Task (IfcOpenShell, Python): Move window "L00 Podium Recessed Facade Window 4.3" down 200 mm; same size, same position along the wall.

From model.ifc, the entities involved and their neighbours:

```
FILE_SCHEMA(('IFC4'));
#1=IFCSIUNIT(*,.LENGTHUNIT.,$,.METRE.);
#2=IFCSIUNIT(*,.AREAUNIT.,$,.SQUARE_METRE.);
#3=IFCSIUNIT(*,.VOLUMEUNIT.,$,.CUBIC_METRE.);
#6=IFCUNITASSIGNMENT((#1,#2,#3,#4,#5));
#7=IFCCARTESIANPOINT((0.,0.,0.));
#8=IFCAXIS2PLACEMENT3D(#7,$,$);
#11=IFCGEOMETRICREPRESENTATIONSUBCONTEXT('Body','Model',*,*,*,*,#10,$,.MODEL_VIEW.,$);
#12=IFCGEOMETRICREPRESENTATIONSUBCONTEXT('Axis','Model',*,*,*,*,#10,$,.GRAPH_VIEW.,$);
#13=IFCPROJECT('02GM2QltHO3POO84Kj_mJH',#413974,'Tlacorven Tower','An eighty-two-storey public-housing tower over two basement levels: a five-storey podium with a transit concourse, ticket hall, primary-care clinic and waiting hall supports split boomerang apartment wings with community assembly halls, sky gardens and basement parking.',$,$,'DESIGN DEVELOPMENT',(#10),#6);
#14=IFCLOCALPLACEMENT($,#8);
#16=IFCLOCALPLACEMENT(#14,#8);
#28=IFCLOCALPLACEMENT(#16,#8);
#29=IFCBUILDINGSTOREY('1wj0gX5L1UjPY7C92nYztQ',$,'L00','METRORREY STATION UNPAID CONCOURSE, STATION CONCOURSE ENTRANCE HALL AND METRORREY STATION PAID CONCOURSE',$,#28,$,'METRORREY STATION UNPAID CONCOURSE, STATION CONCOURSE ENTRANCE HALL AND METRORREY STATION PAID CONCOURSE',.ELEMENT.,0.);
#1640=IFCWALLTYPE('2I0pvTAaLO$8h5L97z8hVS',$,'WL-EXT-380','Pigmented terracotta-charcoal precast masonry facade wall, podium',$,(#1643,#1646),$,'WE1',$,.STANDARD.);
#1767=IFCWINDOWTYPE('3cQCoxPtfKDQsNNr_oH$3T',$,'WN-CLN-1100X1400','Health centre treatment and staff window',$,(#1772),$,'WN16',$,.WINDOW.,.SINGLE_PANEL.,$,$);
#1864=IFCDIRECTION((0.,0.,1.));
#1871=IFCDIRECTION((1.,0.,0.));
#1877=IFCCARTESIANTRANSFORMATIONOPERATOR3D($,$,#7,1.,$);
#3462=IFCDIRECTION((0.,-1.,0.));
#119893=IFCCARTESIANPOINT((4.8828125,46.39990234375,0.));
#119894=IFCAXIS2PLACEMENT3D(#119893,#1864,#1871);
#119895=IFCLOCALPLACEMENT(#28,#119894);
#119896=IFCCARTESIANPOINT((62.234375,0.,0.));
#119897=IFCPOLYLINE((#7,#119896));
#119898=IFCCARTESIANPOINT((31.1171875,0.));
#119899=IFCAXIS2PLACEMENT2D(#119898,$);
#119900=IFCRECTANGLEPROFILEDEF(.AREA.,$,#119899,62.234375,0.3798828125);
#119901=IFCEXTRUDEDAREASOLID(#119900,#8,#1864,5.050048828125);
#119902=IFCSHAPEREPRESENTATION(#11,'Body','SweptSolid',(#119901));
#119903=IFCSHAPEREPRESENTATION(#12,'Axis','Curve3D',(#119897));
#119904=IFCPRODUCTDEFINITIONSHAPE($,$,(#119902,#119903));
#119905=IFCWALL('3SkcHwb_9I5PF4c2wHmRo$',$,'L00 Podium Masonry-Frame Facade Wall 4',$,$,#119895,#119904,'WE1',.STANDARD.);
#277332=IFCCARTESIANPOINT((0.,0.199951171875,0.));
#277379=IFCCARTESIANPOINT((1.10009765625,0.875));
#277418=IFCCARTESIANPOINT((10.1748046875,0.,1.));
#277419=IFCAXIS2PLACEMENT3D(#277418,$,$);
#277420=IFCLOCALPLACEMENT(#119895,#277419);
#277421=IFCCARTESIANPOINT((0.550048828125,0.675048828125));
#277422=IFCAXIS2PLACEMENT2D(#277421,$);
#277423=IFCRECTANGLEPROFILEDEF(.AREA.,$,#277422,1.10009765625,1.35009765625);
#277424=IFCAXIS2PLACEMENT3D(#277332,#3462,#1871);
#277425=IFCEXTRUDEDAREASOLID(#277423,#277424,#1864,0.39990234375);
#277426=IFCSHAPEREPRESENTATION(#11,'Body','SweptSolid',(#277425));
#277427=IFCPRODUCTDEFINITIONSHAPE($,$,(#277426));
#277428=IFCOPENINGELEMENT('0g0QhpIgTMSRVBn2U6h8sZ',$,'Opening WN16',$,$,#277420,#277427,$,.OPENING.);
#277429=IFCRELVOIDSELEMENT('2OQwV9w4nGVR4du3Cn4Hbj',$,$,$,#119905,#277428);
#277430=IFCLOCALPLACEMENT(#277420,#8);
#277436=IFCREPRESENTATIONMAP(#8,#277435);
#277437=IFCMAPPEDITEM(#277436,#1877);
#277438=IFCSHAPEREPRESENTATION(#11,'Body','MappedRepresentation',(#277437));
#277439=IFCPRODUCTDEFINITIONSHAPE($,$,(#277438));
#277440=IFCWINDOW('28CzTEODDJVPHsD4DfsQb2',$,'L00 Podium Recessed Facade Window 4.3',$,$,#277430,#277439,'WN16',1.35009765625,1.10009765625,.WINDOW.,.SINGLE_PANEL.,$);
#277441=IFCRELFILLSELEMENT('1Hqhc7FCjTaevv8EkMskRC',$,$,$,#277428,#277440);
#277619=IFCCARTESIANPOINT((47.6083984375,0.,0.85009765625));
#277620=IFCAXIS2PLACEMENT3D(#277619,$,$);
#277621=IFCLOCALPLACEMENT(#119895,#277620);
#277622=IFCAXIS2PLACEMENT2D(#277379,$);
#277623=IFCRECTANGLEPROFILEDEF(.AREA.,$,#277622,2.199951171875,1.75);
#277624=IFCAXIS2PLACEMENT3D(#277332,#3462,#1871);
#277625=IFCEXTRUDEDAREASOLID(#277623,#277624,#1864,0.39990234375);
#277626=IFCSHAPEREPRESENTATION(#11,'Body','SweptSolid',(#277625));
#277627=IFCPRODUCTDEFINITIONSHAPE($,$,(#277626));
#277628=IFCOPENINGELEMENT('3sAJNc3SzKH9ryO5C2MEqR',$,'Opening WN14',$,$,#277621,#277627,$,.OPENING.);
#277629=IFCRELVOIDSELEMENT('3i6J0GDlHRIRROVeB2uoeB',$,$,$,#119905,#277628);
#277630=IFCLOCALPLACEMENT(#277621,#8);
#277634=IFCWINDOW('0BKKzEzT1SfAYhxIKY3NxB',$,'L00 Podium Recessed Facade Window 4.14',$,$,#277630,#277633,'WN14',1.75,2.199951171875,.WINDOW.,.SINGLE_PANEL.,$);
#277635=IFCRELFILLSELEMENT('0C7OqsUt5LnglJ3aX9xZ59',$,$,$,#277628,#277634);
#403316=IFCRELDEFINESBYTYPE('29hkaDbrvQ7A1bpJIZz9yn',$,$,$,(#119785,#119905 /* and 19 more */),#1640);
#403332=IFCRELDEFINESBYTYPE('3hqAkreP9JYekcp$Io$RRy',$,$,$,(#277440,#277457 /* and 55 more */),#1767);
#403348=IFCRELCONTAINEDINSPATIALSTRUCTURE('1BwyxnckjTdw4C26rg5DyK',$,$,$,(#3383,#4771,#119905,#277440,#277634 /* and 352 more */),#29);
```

```python
import numpy as np
import ifcopenshell
import ifcopenshell.api.geometry
import ifcopenshell.util.placement
import ifcopenshell.util.unit

model = ifcopenshell.open("model.ifc")
unit_scale = ifcopenshell.util.unit.calculate_unit_scale(model)

window = model.by_id(277440)
opening = window.FillsVoids[0].RelatingOpeningElement
dz = -0.2 / unit_scale

shift = np.array([0.0, 0.0, dz])
# The window is placed relative to its opening, so it follows when the opening moves.
matrix = ifcopenshell.util.placement.get_local_placement(opening.ObjectPlacement)
matrix[:3, 3] += shift
ifcopenshell.api.geometry.edit_object_placement(
    model, product=opening, matrix=matrix, is_si=False, should_transform_children=True
)

print(f"moved by {dz * unit_scale:+.3f} m")

model.write("model_rev.ifc")
```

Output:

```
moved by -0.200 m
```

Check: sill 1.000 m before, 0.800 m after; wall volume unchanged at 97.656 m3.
